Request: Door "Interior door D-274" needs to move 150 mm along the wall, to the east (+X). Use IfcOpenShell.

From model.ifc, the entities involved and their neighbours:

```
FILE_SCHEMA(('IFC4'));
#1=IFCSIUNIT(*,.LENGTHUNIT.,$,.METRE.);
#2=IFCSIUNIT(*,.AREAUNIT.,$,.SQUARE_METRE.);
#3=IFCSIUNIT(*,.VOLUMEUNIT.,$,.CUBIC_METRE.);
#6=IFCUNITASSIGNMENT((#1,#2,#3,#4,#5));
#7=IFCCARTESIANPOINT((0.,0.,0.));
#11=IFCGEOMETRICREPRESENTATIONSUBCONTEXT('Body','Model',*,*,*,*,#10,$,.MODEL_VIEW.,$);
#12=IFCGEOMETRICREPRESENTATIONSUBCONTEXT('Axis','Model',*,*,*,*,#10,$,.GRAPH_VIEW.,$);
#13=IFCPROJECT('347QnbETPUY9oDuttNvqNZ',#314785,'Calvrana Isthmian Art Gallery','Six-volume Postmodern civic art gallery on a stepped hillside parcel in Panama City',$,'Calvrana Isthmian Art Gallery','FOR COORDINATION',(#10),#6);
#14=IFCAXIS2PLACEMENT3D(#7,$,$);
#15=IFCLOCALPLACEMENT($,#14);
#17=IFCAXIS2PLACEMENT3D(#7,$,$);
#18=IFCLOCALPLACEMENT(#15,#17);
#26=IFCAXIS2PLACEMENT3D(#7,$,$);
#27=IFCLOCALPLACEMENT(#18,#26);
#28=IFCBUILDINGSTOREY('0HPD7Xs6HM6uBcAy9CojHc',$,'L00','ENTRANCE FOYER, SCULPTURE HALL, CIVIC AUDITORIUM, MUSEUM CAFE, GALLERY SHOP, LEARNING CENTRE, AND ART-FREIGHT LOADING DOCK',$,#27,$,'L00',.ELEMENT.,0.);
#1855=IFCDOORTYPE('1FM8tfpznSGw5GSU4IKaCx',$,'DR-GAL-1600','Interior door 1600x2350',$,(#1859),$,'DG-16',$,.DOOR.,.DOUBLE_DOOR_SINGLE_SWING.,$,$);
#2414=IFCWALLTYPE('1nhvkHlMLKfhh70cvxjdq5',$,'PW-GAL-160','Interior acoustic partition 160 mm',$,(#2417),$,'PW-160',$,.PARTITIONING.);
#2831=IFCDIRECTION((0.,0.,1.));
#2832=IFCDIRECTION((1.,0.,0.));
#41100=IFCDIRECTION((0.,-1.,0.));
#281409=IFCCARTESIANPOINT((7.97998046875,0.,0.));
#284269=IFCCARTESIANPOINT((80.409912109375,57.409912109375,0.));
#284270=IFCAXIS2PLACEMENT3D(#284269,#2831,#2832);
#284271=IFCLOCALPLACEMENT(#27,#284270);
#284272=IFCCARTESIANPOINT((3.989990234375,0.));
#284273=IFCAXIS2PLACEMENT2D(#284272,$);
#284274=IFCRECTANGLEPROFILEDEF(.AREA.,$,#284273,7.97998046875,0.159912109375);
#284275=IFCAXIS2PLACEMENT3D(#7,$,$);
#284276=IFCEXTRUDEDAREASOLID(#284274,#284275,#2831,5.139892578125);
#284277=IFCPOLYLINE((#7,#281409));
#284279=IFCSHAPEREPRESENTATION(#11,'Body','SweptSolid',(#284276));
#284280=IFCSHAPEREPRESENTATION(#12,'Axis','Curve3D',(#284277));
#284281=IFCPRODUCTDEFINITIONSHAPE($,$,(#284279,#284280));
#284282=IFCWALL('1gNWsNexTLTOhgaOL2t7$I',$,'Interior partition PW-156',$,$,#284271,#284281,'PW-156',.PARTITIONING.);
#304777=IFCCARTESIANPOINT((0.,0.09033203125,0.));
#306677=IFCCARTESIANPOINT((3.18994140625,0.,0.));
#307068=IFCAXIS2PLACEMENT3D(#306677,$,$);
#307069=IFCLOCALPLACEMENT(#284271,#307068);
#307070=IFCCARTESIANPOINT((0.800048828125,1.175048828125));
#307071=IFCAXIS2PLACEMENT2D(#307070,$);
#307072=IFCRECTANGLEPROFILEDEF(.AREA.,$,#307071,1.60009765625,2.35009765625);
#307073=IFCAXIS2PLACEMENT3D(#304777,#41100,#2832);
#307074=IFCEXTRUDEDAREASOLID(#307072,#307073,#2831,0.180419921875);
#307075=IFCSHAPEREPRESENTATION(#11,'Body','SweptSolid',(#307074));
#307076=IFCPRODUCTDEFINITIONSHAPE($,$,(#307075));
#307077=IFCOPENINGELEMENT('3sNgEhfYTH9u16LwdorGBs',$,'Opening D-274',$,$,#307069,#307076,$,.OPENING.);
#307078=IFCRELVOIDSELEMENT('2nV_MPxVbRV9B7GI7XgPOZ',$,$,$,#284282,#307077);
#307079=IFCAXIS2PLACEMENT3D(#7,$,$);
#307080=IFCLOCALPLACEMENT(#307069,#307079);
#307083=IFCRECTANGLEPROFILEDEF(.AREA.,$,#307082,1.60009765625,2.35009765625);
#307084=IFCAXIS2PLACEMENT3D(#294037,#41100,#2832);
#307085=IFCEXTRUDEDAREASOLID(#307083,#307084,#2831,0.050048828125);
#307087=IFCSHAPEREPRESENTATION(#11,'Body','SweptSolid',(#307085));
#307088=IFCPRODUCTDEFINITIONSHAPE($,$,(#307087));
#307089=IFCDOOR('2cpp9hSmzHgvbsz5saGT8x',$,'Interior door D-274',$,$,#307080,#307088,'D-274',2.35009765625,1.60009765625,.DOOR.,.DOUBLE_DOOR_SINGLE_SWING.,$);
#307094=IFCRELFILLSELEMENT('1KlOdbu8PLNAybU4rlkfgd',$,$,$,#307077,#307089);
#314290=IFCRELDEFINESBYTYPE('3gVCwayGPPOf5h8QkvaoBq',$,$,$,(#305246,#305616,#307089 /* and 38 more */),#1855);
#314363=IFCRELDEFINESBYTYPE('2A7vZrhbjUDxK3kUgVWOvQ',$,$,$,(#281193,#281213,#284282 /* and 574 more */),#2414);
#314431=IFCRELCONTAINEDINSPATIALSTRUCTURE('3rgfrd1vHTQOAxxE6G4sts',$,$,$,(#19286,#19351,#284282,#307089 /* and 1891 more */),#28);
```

```python
import ifcopenshell
import ifcopenshell.api.geometry
import ifcopenshell.util.placement

model = ifcopenshell.open("model.ifc")

door = model.by_guid("2cpp9hSmzHgvbsz5saGT8x")
opening = door.FillsVoids[0].RelatingOpeningElement
wall = opening.VoidsElements[0].RelatingBuildingElement

wall_matrix = ifcopenshell.util.placement.get_local_placement(wall.ObjectPlacement)
shift = wall_matrix[:3, 0] * 0.15
before = ifcopenshell.util.placement.get_local_placement(door.ObjectPlacement)[:3, 3].copy()

# The door is placed relative to its opening, so it follows when the opening moves.
matrix = ifcopenshell.util.placement.get_local_placement(opening.ObjectPlacement)
matrix[:3, 3] += shift
ifcopenshell.api.geometry.edit_object_placement(
    model, product=opening, matrix=matrix, is_si=False, should_transform_children=True
)

after = ifcopenshell.util.placement.get_local_placement(door.ObjectPlacement)[:3, 3]
print("door moved by", (after - before).round(3) + 0.0)

model.write("model_rev.ifc")
```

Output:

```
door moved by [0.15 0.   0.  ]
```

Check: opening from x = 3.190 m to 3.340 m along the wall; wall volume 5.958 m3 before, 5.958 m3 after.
